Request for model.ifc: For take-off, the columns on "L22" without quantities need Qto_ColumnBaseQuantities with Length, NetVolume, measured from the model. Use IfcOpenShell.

First a look at what the model holds.

```python
import ifcopenshell
import ifcopenshell.util.element
import ifcopenshell.util.unit

model = ifcopenshell.open("model.ifc")
print(model.schema)
for unit_type in ("LENGTHUNIT", "AREAUNIT", "VOLUMEUNIT"):
    print(unit_type, ifcopenshell.util.unit.calculate_unit_scale(model, unit_type))
storey = next(s for s in model.by_type("IfcBuildingStorey") if s.Name == "L22")
columns = [e for e in ifcopenshell.util.element.get_decomposition(storey) if e.is_a("IfcColumn")]
for e in sorted(columns, key=lambda e: e.id()):
    print(e.id(), e.is_a(), e.Name, list(ifcopenshell.util.element.get_psets(e, qtos_only=True)), sep=" | ")
```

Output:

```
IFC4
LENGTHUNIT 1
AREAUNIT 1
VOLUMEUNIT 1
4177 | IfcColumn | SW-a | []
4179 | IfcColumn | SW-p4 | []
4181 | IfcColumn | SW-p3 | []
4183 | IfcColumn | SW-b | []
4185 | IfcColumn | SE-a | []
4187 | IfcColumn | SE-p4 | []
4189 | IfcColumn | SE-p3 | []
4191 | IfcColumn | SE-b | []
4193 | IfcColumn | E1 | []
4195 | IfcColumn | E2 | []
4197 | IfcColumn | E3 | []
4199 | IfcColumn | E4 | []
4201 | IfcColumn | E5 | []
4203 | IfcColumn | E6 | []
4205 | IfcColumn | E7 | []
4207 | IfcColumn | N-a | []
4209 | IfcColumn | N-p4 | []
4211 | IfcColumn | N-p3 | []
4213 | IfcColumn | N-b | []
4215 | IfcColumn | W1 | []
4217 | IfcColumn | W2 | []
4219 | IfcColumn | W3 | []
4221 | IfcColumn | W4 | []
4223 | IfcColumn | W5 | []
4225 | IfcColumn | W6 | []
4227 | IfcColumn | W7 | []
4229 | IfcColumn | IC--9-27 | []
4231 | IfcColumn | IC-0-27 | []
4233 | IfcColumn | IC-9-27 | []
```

```python
import ifcopenshell
import ifcopenshell.api.pset
import ifcopenshell.geom
import ifcopenshell.util.element
import ifcopenshell.util.shape
import ifcopenshell.util.unit

model = ifcopenshell.open("model.ifc")
unit_scale = ifcopenshell.util.unit.calculate_unit_scale(model)
volume_scale = ifcopenshell.util.unit.calculate_unit_scale(model, "VOLUMEUNIT")
settings = ifcopenshell.geom.settings()

storey = next(s for s in model.by_type("IfcBuildingStorey") if s.Name == "L22")
columns = [e for e in ifcopenshell.util.element.get_decomposition(storey) if e.is_a("IfcColumn")]

for e in sorted(columns, key=lambda e: e.id()):
    if ifcopenshell.util.element.get_psets(e, qtos_only=True, should_inherit=False):
        continue
    # Geometry comes back in metres, in the element's own axes.
    shape = ifcopenshell.geom.create_shape(settings, e)
    values = {
        "Length": ifcopenshell.util.shape.get_z(shape.geometry) / unit_scale,
        "NetVolume": ifcopenshell.util.shape.get_volume(shape.geometry) / volume_scale,
    }
    qto = ifcopenshell.api.pset.add_qto(model, product=e, name="Qto_ColumnBaseQuantities")
    ifcopenshell.api.pset.edit_qto(model, qto=qto, properties=values)
    print(e.id(), {k: round(v, 3) for k, v in values.items()})

model.write("model-out.ifc")
```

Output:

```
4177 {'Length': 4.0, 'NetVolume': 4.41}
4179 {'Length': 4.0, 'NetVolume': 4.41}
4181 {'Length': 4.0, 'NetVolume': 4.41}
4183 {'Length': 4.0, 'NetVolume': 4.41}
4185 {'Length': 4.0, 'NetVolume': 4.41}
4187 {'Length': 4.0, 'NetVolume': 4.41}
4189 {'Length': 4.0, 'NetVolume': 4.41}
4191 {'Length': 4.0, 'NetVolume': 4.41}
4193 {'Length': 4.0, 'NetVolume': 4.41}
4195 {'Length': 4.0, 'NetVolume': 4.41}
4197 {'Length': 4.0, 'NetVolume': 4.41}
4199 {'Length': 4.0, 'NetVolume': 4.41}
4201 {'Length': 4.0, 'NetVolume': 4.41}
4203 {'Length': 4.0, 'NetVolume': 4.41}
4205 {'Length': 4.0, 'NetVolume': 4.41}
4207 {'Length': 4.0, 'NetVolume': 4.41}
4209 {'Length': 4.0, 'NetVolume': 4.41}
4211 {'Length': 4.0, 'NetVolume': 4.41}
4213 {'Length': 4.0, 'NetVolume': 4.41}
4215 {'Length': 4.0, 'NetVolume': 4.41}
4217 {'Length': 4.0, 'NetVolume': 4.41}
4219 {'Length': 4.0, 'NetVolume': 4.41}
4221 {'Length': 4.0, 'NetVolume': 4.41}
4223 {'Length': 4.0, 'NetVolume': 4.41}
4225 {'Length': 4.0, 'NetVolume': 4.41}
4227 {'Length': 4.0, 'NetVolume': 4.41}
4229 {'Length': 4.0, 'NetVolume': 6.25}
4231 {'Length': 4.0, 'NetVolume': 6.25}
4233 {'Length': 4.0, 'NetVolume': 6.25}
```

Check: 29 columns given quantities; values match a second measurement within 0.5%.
